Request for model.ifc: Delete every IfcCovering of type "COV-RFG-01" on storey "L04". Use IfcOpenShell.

First a look at what the model holds.

```python
import ifcopenshell
import ifcopenshell.util.element

model = ifcopenshell.open("model.ifc")
print(model.schema)
storey = next(s for s in model.by_type("IfcBuildingStorey") if s.Name == "L04")
coverings = [e for e in ifcopenshell.util.element.get_decomposition(storey) if e.is_a("IfcCovering")]
seen = {}
for e in coverings:
    element_type = ifcopenshell.util.element.get_type(e)
    name = element_type.Name if element_type not in (None, e) else None
    seen[name] = seen.get(name, 0) + 1
for name, count in sorted(seen.items(), key=str):
    print(count, "x", name)
```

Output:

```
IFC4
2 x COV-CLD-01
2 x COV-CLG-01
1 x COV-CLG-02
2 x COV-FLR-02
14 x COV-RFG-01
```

```python
import ifcopenshell
import ifcopenshell.api.root
import ifcopenshell.util.element

model = ifcopenshell.open("model.ifc")

storey = next(s for s in model.by_type("IfcBuildingStorey") if s.Name == "L04")
coverings = [e for e in ifcopenshell.util.element.get_decomposition(storey) if e.is_a("IfcCovering")]
targets = [e for e in coverings if (t := ifcopenshell.util.element.get_type(e)) not in (None, e) and t.Name == "COV-RFG-01"]

for e in targets:
    ifcopenshell.api.root.remove_product(model, product=e)
print(len(targets), "removed")

model.write("model_edited.ifc")
```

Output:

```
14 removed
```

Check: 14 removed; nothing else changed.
